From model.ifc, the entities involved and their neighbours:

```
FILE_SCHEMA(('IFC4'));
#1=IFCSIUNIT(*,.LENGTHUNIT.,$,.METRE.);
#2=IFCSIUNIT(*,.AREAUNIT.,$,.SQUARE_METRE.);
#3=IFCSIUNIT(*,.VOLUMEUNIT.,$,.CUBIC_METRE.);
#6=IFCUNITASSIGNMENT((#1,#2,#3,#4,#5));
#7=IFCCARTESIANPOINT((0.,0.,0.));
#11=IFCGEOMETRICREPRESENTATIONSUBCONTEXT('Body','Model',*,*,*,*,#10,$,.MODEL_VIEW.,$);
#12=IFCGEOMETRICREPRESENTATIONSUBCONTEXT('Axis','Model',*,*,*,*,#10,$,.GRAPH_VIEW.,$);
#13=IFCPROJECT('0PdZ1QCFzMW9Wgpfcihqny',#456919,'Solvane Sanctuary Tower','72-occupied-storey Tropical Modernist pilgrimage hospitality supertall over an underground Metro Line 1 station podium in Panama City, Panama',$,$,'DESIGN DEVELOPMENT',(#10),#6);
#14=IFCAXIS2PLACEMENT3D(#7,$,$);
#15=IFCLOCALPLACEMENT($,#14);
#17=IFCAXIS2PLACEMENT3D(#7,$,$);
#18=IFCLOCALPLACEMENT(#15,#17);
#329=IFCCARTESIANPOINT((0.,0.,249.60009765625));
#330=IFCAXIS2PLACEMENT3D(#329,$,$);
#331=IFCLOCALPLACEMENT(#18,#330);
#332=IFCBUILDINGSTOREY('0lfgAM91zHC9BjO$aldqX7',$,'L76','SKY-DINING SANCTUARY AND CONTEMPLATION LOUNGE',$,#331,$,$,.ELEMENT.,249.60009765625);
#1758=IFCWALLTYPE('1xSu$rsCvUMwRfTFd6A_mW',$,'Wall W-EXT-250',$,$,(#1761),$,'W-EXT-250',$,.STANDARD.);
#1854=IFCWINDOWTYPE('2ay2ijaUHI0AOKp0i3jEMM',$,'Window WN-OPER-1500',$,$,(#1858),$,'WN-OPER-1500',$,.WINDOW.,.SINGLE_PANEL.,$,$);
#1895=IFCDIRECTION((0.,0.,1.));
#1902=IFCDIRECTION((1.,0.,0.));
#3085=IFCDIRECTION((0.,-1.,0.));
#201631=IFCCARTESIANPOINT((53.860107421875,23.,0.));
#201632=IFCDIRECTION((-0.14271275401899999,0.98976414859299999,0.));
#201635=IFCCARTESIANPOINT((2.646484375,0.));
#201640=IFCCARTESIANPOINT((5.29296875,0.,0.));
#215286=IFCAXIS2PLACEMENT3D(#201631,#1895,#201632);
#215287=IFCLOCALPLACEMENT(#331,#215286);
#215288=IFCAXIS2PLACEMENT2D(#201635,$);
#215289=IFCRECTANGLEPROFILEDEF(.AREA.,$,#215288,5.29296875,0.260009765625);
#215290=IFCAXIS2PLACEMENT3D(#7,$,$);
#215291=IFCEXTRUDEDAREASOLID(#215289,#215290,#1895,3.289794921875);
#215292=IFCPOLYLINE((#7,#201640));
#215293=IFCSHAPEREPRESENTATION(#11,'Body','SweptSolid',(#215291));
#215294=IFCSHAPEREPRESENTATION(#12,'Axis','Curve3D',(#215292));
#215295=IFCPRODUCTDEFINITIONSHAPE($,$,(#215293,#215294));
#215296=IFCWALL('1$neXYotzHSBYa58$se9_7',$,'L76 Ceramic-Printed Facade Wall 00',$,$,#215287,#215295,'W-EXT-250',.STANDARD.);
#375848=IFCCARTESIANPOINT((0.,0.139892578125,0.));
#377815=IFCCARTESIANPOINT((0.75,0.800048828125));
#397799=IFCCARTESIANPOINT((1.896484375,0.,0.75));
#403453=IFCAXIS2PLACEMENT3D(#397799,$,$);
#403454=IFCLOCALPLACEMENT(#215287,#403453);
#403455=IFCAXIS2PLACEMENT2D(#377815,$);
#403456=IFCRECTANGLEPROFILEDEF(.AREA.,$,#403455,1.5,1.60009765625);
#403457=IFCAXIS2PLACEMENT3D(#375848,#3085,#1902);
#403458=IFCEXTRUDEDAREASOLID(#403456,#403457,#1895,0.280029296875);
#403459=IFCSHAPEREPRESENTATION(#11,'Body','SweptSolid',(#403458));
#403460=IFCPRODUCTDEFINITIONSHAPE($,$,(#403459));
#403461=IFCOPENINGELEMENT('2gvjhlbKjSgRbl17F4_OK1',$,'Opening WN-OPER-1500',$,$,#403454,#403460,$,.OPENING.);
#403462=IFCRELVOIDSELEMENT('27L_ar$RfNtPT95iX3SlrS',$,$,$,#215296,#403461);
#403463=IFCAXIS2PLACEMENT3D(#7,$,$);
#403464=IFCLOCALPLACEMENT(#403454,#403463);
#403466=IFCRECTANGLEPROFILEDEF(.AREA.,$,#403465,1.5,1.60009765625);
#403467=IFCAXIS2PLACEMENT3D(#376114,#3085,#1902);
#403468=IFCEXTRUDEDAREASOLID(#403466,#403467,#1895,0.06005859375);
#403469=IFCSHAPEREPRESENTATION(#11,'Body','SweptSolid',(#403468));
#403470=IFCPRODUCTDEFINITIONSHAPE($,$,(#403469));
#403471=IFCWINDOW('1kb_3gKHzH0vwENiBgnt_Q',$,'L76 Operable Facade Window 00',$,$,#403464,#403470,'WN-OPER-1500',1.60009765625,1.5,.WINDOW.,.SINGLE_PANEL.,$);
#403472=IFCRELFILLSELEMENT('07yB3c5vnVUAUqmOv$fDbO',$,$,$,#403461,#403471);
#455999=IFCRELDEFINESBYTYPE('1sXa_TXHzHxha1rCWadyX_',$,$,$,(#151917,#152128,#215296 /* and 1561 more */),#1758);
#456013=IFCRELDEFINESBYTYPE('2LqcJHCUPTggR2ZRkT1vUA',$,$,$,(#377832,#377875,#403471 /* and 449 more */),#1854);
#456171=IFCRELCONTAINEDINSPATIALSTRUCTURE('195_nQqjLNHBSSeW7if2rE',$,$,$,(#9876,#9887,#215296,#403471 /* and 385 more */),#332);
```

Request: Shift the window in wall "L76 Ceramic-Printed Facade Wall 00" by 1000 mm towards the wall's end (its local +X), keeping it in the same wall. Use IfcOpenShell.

```python
import ifcopenshell
import ifcopenshell.api.geometry
import ifcopenshell.util.placement
import ifcopenshell.util.unit

model = ifcopenshell.open("model.ifc")
unit_scale = ifcopenshell.util.unit.calculate_unit_scale(model)

window = model.by_guid("1kb_3gKHzH0vwENiBgnt_Q")
opening = window.FillsVoids[0].RelatingOpeningElement
wall = opening.VoidsElements[0].RelatingBuildingElement

wall_matrix = ifcopenshell.util.placement.get_local_placement(wall.ObjectPlacement)
shift = wall_matrix[:3, 0] * 1 / unit_scale
before = ifcopenshell.util.placement.get_local_placement(window.ObjectPlacement)[:3, 3].copy()

# The window is placed relative to its opening, so it follows when the opening moves.
matrix = ifcopenshell.util.placement.get_local_placement(opening.ObjectPlacement)
matrix[:3, 3] += shift
ifcopenshell.api.geometry.edit_object_placement(
    model, product=opening, matrix=matrix, is_si=False, should_transform_children=True
)

after = ifcopenshell.util.placement.get_local_placement(window.ObjectPlacement)[:3, 3]
print("window moved by", (after - before).round(3) + 0.0)

model.write("model_edited.ifc")
```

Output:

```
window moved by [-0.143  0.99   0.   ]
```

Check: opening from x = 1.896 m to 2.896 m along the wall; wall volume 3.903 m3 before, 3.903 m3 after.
